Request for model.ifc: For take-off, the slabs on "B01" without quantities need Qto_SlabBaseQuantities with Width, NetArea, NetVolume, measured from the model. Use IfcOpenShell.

First a look at what the model holds.

```python
import ifcopenshell
import ifcopenshell.util.element
import ifcopenshell.util.unit

model = ifcopenshell.open("model.ifc")
print(model.schema)
for unit_type in ("LENGTHUNIT", "AREAUNIT", "VOLUMEUNIT"):
    print(unit_type, ifcopenshell.util.unit.calculate_unit_scale(model, unit_type))
storey = next(s for s in model.by_type("IfcBuildingStorey") if s.Name == "B01")
slabs = [e for e in ifcopenshell.util.element.get_decomposition(storey) if e.is_a("IfcSlab")]
for e in sorted(slabs, key=lambda e: e.id()):
    print(e.id(), e.is_a(), e.Name, list(ifcopenshell.util.element.get_psets(e, qtos_only=True)), sep=" | ")
```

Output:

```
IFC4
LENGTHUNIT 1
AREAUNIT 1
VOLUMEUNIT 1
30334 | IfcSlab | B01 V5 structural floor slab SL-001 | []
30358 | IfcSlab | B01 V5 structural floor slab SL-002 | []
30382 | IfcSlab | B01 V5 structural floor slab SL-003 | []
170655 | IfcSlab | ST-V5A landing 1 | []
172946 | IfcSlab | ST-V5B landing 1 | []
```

```python
import ifcopenshell
import ifcopenshell.api.pset
import ifcopenshell.geom
import ifcopenshell.util.element
import ifcopenshell.util.shape
import ifcopenshell.util.unit

model = ifcopenshell.open("model.ifc")
unit_scale = ifcopenshell.util.unit.calculate_unit_scale(model)
area_scale = ifcopenshell.util.unit.calculate_unit_scale(model, "AREAUNIT")
volume_scale = ifcopenshell.util.unit.calculate_unit_scale(model, "VOLUMEUNIT")
settings = ifcopenshell.geom.settings()

storey = next(s for s in model.by_type("IfcBuildingStorey") if s.Name == "B01")
slabs = [e for e in ifcopenshell.util.element.get_decomposition(storey) if e.is_a("IfcSlab")]

for e in sorted(slabs, key=lambda e: e.id()):
    if ifcopenshell.util.element.get_psets(e, qtos_only=True, should_inherit=False):
        continue
    # Geometry comes back in metres, in the element's own axes.
    shape = ifcopenshell.geom.create_shape(settings, e)
    values = {
        "Width": ifcopenshell.util.shape.get_z(shape.geometry) / unit_scale,
        "NetArea": ifcopenshell.util.shape.get_footprint_area(shape.geometry) / area_scale,
        "NetVolume": ifcopenshell.util.shape.get_volume(shape.geometry) / volume_scale,
    }
    qto = ifcopenshell.api.pset.add_qto(model, product=e, name="Qto_SlabBaseQuantities")
    ifcopenshell.api.pset.edit_qto(model, qto=qto, properties=values)
    print(e.id(), {k: round(v, 3) for k, v in values.items()})

model.write("model-out.ifc")
```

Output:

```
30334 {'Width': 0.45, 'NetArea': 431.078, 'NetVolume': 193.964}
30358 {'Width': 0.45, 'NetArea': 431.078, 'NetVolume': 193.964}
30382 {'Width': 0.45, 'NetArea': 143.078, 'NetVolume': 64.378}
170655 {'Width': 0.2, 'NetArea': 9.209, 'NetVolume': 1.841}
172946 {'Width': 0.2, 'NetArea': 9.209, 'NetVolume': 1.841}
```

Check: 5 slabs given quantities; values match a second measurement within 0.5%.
